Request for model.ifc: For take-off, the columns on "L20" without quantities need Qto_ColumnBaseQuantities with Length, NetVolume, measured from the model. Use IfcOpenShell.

First a look at what the model holds.

```python
import ifcopenshell
import ifcopenshell.util.element
import ifcopenshell.util.unit

model = ifcopenshell.open("model.ifc")
print(model.schema)
for unit_type in ("LENGTHUNIT", "AREAUNIT", "VOLUMEUNIT"):
    print(unit_type, ifcopenshell.util.unit.calculate_unit_scale(model, unit_type))
storey = next(s for s in model.by_type("IfcBuildingStorey") if s.Name == "L20")
columns = [e for e in ifcopenshell.util.element.get_decomposition(storey) if e.is_a("IfcColumn")]
for e in sorted(columns, key=lambda e: e.id()):
    print(e.id(), e.is_a(), e.Name, list(ifcopenshell.util.element.get_psets(e, qtos_only=True)), sep=" | ")
```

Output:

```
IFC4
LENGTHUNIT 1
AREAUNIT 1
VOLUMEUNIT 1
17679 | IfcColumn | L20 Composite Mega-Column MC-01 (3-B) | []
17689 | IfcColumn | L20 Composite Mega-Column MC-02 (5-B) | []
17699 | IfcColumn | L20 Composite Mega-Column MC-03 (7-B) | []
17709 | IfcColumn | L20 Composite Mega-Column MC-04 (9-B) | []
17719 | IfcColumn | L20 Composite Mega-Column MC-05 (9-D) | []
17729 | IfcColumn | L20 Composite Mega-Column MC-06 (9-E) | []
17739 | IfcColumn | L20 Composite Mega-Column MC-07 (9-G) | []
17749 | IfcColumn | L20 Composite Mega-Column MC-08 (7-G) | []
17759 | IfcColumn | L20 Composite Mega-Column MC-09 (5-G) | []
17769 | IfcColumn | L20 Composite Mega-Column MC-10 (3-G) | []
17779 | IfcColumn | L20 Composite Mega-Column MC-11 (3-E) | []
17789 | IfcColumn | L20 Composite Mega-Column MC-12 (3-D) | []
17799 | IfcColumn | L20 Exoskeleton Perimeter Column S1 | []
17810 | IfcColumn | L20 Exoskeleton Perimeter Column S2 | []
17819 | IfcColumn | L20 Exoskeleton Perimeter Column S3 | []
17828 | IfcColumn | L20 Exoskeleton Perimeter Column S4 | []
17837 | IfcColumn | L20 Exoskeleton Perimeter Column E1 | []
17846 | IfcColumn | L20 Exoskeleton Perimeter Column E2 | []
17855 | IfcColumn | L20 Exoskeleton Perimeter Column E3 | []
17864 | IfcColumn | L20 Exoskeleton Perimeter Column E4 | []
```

```python
import ifcopenshell
import ifcopenshell.api.pset
import ifcopenshell.geom
import ifcopenshell.util.element
import ifcopenshell.util.shape
import ifcopenshell.util.unit

model = ifcopenshell.open("model.ifc")
unit_scale = ifcopenshell.util.unit.calculate_unit_scale(model)
volume_scale = ifcopenshell.util.unit.calculate_unit_scale(model, "VOLUMEUNIT")
settings = ifcopenshell.geom.settings()

storey = next(s for s in model.by_type("IfcBuildingStorey") if s.Name == "L20")
columns = [e for e in ifcopenshell.util.element.get_decomposition(storey) if e.is_a("IfcColumn")]

for e in sorted(columns, key=lambda e: e.id()):
    if ifcopenshell.util.element.get_psets(e, qtos_only=True, should_inherit=False):
        continue
    # Geometry comes back in metres, in the element's own axes.
    shape = ifcopenshell.geom.create_shape(settings, e)
    values = {
        "Length": ifcopenshell.util.shape.get_z(shape.geometry) / unit_scale,
        "NetVolume": ifcopenshell.util.shape.get_volume(shape.geometry) / volume_scale,
    }
    qto = ifcopenshell.api.pset.add_qto(model, product=e, name="Qto_ColumnBaseQuantities")
    ifcopenshell.api.pset.edit_qto(model, qto=qto, properties=values)
    print(e.id(), {k: round(v, 3) for k, v in values.items()})

model.write("model_v2.ifc")
```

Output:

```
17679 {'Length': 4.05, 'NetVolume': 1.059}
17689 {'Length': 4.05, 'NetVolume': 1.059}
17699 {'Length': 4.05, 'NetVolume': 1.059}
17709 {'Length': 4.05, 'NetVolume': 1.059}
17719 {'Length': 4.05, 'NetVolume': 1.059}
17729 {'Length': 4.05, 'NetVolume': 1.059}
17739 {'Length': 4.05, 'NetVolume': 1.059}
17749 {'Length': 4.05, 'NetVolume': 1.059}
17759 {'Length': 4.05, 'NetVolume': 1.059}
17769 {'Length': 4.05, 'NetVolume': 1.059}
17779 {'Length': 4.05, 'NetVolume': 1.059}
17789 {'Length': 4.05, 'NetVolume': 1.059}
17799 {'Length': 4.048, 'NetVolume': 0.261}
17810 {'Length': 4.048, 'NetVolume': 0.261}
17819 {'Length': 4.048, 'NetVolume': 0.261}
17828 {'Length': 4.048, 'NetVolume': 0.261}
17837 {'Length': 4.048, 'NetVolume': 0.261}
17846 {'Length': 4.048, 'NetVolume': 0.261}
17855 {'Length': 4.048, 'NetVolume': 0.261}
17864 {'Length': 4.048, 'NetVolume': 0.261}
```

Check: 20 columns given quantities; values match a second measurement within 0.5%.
